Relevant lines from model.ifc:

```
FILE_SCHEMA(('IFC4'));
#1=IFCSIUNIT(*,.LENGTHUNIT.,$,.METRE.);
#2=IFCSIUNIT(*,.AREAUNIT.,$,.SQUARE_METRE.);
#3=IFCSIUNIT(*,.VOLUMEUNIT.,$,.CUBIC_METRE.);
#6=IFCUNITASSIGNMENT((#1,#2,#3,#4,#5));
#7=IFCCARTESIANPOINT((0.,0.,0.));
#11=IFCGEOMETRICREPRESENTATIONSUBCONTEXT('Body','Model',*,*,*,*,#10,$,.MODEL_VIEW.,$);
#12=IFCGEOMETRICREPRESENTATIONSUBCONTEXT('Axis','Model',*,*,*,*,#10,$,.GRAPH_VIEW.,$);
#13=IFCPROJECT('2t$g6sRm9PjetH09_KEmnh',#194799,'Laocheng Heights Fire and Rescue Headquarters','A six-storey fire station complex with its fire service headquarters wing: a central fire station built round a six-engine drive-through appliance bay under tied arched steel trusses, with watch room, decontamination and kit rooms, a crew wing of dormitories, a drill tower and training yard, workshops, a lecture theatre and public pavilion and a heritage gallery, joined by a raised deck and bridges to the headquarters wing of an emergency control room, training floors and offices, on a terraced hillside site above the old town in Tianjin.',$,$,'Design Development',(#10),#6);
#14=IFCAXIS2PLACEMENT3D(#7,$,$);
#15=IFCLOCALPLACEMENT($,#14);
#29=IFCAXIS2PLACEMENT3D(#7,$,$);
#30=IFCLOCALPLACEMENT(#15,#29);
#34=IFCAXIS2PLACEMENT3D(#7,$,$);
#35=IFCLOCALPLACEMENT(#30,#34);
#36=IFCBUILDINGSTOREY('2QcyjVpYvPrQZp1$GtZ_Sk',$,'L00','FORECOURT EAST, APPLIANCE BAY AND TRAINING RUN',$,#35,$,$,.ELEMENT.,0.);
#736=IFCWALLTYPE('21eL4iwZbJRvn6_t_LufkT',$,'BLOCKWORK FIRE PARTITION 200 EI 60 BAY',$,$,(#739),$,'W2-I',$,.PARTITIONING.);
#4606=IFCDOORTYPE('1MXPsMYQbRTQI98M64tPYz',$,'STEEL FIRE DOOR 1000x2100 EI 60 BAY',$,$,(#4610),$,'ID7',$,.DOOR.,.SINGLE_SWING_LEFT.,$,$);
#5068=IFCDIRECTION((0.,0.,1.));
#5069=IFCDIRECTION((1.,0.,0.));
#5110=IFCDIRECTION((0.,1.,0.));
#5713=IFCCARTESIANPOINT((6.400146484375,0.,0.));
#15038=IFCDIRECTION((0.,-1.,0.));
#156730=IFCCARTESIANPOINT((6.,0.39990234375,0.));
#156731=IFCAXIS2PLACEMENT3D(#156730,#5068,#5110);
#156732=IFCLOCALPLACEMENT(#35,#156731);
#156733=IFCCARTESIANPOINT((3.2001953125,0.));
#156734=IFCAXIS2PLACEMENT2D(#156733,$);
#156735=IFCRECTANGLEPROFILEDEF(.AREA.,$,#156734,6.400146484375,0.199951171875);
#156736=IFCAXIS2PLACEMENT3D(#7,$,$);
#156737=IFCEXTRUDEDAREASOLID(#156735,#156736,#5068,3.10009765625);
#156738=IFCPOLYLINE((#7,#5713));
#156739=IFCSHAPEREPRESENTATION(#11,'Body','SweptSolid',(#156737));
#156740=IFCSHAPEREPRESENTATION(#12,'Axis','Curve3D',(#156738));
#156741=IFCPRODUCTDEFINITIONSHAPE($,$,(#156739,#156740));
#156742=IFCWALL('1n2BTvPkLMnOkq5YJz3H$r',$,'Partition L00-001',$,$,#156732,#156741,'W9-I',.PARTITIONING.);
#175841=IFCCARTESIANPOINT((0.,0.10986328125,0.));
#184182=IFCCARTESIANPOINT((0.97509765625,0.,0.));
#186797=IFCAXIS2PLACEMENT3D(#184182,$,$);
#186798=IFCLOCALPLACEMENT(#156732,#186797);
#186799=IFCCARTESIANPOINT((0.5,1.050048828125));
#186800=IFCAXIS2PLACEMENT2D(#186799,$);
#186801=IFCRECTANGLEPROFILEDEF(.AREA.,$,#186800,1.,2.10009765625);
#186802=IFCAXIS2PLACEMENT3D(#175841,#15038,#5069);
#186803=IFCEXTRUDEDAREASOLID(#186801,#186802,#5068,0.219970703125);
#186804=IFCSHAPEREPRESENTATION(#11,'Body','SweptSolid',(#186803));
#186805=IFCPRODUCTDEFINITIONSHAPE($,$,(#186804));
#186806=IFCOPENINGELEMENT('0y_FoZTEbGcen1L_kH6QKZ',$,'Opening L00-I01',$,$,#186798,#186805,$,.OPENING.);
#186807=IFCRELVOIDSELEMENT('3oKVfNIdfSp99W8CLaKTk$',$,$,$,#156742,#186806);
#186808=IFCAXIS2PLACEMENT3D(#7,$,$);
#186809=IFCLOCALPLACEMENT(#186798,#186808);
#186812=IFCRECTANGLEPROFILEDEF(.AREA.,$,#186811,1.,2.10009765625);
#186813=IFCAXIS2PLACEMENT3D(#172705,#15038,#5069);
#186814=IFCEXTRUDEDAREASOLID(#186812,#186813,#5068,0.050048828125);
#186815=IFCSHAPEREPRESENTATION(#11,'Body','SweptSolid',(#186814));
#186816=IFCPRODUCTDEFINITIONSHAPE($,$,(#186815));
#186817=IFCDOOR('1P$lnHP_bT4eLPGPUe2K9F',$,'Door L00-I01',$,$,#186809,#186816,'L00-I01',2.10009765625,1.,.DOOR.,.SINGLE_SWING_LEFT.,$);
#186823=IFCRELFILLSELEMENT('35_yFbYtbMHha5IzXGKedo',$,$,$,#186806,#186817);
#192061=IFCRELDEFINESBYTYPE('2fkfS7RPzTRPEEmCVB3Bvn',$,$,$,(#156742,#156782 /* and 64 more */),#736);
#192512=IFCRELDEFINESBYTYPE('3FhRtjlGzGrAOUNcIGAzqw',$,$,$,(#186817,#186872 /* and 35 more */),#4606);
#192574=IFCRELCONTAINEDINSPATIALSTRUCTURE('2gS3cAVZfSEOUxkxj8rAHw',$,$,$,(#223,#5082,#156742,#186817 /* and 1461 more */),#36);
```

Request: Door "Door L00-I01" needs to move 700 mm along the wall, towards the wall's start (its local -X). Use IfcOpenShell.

```python
import ifcopenshell
import ifcopenshell.api.geometry
import ifcopenshell.util.placement
import ifcopenshell.util.unit

model = ifcopenshell.open("model.ifc")
unit_scale = ifcopenshell.util.unit.calculate_unit_scale(model)

door = model.by_guid("1P$lnHP_bT4eLPGPUe2K9F")
opening = door.FillsVoids[0].RelatingOpeningElement
wall = opening.VoidsElements[0].RelatingBuildingElement

wall_matrix = ifcopenshell.util.placement.get_local_placement(wall.ObjectPlacement)
shift = wall_matrix[:3, 0] * -0.7 / unit_scale
before = ifcopenshell.util.placement.get_local_placement(door.ObjectPlacement)[:3, 3].copy()

# The door is placed relative to its opening, so it follows when the opening moves.
matrix = ifcopenshell.util.placement.get_local_placement(opening.ObjectPlacement)
matrix[:3, 3] += shift
ifcopenshell.api.geometry.edit_object_placement(
    model, product=opening, matrix=matrix, is_si=False, should_transform_children=True
)

after = ifcopenshell.util.placement.get_local_placement(door.ObjectPlacement)[:3, 3]
print("door moved by", (after - before).round(3) + 0.0)

model.write("model_edited.ifc")
```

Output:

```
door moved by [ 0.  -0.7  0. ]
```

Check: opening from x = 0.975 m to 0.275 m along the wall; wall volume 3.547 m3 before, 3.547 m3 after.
